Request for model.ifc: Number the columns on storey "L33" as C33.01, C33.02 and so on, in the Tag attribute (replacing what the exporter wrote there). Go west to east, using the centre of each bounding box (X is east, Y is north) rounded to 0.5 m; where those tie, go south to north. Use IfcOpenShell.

First a look at what the model holds.

```python
import ifcopenshell
import ifcopenshell.util.element
import ifcopenshell.util.placement

model = ifcopenshell.open("model.ifc")
print(model.schema)
storey = next(s for s in model.by_type("IfcBuildingStorey") if s.Name == "L33")
columns = [e for e in ifcopenshell.util.element.get_decomposition(storey) if e.is_a("IfcColumn")]
for e in sorted(columns, key=lambda e: e.id()):
    origin = ifcopenshell.util.placement.get_local_placement(e.ObjectPlacement)[:3, 3]
    print(e.id(), e.Tag, e.Name, origin.round(2) + 0.0, sep=" | ")
```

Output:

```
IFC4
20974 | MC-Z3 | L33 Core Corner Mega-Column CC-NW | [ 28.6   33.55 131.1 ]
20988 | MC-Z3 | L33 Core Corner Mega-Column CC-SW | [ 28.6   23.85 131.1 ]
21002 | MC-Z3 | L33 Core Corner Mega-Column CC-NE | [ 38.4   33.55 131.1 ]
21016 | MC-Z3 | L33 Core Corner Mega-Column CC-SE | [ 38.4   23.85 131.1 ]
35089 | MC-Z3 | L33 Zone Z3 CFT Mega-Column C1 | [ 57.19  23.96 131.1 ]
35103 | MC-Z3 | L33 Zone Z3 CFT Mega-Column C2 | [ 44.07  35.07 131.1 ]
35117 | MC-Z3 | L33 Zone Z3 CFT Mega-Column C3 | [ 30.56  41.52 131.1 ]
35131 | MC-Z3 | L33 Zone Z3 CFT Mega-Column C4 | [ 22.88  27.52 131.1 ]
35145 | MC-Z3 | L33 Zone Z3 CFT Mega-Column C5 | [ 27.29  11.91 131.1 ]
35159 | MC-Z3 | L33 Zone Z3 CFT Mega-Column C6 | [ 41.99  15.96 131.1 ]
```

```python
import ifcopenshell
import ifcopenshell.geom
import ifcopenshell.util.element
import ifcopenshell.util.shape

model = ifcopenshell.open("model.ifc")
settings = ifcopenshell.geom.settings()
settings.set("use-world-coords", True)


def centre(element):
    shape = ifcopenshell.geom.create_shape(settings, element)
    return ifcopenshell.util.shape.get_bbox_centroid(shape.geometry)


storey = next(s for s in model.by_type("IfcBuildingStorey") if s.Name == "L33")
columns = [e for e in ifcopenshell.util.element.get_decomposition(storey) if e.is_a("IfcColumn")]

# Insertion points can sit at a corner or the storey origin, so sort by the geometry (in metres).
centres = {e: centre(e) for e in columns}
columns.sort(key=lambda e: (round(centres[e][0] / 0.5), centres[e][1]))

for i, e in enumerate(columns, start=1):
    number = f"C33.{i:02d}"
    e.Tag = number
    print(e.id(), number)

model.write("model_v2.ifc")
```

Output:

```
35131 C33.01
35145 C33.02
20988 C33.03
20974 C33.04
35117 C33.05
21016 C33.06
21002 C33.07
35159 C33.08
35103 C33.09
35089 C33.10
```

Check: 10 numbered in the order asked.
